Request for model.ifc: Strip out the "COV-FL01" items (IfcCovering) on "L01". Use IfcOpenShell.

First a look at what the model holds.

```python
import ifcopenshell
import ifcopenshell.util.element

model = ifcopenshell.open("model.ifc")
print(model.schema)
storey = next(s for s in model.by_type("IfcBuildingStorey") if s.Name == "L01")
coverings = [e for e in ifcopenshell.util.element.get_decomposition(storey) if e.is_a("IfcCovering")]
seen = {}
for e in coverings:
    element_type = ifcopenshell.util.element.get_type(e)
    name = element_type.Name if element_type not in (None, e) else None
    seen[name] = seen.get(name, 0) + 1
for name, count in sorted(seen.items(), key=str):
    print(count, "x", name)
```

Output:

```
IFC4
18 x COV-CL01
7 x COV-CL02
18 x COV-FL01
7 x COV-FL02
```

```python
import ifcopenshell
import ifcopenshell.api.root
import ifcopenshell.util.element

model = ifcopenshell.open("model.ifc")

storey = next(s for s in model.by_type("IfcBuildingStorey") if s.Name == "L01")
coverings = [e for e in ifcopenshell.util.element.get_decomposition(storey) if e.is_a("IfcCovering")]
targets = [e for e in coverings if (t := ifcopenshell.util.element.get_type(e)) not in (None, e) and t.Name == "COV-FL01"]

for e in targets:
    ifcopenshell.api.root.remove_product(model, product=e)
print(len(targets), "removed")

model.write("model_rev.ifc")
```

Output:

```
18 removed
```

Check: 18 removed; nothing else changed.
